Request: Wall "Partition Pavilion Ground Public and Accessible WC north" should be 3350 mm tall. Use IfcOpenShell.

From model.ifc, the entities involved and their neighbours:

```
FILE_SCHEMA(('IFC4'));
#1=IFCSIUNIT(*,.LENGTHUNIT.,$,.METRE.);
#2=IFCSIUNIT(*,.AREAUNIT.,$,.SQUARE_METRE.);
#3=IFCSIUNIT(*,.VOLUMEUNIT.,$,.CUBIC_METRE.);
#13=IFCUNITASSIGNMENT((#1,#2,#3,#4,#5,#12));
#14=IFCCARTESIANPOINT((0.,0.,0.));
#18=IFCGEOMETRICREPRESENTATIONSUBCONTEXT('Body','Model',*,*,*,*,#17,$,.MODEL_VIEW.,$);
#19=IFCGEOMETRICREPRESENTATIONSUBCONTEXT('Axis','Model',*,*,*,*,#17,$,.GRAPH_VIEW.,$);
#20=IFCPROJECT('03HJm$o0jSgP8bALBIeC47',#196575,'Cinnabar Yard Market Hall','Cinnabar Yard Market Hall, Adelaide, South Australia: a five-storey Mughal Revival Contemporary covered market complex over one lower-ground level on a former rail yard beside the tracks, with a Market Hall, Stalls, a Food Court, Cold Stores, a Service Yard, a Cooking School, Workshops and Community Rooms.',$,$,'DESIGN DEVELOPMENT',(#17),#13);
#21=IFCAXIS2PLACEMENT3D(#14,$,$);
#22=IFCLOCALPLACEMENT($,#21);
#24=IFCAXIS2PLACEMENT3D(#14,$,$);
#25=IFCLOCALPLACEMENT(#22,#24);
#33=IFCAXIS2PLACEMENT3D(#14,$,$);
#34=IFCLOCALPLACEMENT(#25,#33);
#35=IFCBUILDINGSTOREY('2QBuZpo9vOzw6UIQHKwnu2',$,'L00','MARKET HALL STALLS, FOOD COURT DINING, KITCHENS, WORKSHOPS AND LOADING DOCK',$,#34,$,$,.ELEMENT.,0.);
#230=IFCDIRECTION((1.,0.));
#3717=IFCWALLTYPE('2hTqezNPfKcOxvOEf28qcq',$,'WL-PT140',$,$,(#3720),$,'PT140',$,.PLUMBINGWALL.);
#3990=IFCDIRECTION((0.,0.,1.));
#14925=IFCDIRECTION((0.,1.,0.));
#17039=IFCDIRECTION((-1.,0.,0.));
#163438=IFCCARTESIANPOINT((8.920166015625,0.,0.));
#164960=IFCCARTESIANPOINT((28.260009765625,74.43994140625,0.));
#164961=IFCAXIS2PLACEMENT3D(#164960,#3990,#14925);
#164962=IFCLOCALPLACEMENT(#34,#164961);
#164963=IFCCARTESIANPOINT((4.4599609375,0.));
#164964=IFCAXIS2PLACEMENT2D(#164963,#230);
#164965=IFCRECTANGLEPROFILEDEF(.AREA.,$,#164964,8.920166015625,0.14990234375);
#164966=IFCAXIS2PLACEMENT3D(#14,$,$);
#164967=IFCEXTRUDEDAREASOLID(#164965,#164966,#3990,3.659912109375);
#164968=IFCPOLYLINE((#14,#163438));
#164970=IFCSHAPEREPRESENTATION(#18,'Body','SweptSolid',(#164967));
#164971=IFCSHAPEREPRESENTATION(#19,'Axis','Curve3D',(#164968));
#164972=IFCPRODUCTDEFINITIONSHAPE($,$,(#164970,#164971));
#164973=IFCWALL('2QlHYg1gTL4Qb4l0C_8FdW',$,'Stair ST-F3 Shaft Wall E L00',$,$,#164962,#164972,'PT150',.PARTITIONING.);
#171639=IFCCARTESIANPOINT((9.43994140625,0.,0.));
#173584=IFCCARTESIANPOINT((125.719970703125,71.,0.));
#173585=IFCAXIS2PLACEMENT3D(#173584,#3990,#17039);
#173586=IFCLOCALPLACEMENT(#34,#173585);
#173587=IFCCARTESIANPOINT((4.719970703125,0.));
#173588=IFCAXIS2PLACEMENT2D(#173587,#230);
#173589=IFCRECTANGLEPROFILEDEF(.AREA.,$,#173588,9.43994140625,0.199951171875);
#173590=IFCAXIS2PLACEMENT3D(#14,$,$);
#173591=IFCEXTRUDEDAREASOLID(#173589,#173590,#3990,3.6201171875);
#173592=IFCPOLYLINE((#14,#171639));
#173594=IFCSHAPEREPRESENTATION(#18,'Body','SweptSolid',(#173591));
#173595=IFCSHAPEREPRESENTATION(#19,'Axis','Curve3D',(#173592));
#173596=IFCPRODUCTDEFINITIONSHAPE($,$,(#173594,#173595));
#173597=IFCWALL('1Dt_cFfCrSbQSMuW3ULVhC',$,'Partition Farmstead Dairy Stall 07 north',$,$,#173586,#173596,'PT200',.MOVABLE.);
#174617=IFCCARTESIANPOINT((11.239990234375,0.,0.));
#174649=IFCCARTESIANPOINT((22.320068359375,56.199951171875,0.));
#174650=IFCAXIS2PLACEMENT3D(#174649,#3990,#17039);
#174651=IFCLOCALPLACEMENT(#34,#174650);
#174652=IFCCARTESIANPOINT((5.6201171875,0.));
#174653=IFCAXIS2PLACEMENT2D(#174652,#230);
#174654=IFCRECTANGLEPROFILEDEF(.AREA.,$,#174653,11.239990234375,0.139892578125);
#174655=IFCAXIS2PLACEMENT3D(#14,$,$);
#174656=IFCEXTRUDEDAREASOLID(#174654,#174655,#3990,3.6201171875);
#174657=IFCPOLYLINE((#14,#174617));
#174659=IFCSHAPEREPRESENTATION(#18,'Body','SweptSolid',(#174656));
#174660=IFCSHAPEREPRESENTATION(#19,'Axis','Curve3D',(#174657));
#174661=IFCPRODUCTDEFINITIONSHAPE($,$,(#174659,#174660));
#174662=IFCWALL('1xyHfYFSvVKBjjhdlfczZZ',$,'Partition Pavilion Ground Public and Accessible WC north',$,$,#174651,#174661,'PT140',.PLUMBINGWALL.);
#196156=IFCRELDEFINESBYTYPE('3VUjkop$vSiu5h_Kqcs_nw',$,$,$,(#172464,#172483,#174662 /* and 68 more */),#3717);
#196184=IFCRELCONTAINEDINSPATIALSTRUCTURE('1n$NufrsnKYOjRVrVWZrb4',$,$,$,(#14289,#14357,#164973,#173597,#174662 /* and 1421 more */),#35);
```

```python
import ifcopenshell
import ifcopenshell.geom
import ifcopenshell.util.representation
import ifcopenshell.util.shape

model = ifcopenshell.open("model.ifc")
settings = ifcopenshell.geom.settings()


def volume(element):
    """Net volume in cubic metres, openings subtracted."""
    shape = ifcopenshell.geom.create_shape(settings, element)
    return ifcopenshell.util.shape.get_volume(shape.geometry)


wall = model.by_guid("1xyHfYFSvVKBjjhdlfczZZ")
before = volume(wall)

body = ifcopenshell.util.representation.get_representation(wall, "Model", "Body")
solid = body.Items[0]
old_height = solid.Depth
solid.Depth = 3.35
after = volume(wall)

print(f"height {old_height:g} -> {solid.Depth:g}, volume {before:.3f} -> {after:.3f} m3")

model.write("model-out.ifc")
```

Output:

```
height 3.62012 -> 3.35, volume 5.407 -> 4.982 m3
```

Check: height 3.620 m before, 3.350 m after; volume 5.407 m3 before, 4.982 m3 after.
